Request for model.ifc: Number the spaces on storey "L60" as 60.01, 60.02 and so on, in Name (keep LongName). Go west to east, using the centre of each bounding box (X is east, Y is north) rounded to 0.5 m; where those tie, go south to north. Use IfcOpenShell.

First a look at what the model holds.

```python
import ifcopenshell
import ifcopenshell.util.element
import ifcopenshell.util.placement

model = ifcopenshell.open("model.ifc")
print(model.schema)
storey = next(s for s in model.by_type("IfcBuildingStorey") if s.Name == "L60")
spaces = [e for e in ifcopenshell.util.element.get_decomposition(storey) if e.is_a("IfcSpace")]
for e in sorted(spaces, key=lambda e: e.id()):
    origin = ifcopenshell.util.placement.get_local_placement(e.ObjectPlacement)[:3, 3]
    print(e.id(), e.Name, e.LongName, origin.round(2) + 0.0, sep=" | ")
```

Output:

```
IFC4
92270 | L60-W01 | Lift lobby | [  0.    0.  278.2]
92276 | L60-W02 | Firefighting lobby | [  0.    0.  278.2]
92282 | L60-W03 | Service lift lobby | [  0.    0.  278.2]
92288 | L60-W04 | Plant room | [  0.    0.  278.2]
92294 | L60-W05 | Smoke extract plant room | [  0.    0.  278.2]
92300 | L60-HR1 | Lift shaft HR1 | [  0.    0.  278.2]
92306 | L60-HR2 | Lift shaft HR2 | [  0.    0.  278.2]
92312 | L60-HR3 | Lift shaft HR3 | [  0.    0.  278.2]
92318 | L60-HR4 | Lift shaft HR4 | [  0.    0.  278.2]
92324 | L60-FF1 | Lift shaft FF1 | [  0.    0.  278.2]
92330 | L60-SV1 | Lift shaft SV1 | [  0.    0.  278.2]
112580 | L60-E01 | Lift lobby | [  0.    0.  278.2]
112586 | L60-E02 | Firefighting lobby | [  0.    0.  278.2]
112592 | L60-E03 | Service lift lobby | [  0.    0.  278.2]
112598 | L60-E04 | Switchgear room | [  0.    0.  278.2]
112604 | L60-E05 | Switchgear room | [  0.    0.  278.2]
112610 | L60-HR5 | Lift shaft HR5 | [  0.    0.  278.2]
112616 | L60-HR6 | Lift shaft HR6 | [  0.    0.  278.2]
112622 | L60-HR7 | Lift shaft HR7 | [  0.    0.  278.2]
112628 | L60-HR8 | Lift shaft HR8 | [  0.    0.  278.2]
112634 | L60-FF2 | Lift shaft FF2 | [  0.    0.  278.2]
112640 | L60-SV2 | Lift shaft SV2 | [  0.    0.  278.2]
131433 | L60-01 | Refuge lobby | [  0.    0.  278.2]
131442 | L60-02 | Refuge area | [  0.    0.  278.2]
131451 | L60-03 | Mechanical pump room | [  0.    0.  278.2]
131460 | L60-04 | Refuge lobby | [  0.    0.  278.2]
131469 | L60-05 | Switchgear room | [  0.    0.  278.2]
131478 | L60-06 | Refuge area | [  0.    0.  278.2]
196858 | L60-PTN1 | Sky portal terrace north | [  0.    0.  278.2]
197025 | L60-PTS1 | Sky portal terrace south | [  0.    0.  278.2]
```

```python
import ifcopenshell
import ifcopenshell.geom
import ifcopenshell.util.element
import ifcopenshell.util.shape

model = ifcopenshell.open("model.ifc")
settings = ifcopenshell.geom.settings()
settings.set("use-world-coords", True)


def centre(element):
    shape = ifcopenshell.geom.create_shape(settings, element)
    return ifcopenshell.util.shape.get_bbox_centroid(shape.geometry)


storey = next(s for s in model.by_type("IfcBuildingStorey") if s.Name == "L60")
spaces = [e for e in ifcopenshell.util.element.get_decomposition(storey) if e.is_a("IfcSpace")]

# Insertion points can sit at a corner or the storey origin, so sort by the geometry (in metres).
centres = {e: centre(e) for e in spaces}
spaces.sort(key=lambda e: (round(centres[e][0] / 0.5), centres[e][1]))

for i, e in enumerate(spaces, start=1):
    number = f"60.{i:02d}"
    e.Name = number
    print(e.id(), number)

model.write("model_v2.ifc")
```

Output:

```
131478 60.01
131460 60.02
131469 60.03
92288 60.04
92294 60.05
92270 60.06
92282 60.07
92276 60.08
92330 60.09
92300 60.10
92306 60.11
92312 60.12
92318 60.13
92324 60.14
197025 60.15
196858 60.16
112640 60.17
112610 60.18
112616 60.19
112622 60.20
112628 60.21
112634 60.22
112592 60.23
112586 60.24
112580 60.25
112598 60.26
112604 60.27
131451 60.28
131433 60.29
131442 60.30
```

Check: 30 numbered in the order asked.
